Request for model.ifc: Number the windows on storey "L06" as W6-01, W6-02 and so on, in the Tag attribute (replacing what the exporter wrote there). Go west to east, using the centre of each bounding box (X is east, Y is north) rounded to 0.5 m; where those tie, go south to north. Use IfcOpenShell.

First a look at what the model holds.

```python
import ifcopenshell
import ifcopenshell.util.element
import ifcopenshell.util.placement

model = ifcopenshell.open("model.ifc")
print(model.schema)
storey = next(s for s in model.by_type("IfcBuildingStorey") if s.Name == "L06")
windows = [e for e in ifcopenshell.util.element.get_decomposition(storey) if e.is_a("IfcWindow")]
for e in sorted(windows, key=lambda e: e.id()):
    origin = ifcopenshell.util.placement.get_local_placement(e.ObjectPlacement)[:3, 3]
    print(e.id(), e.Tag, e.Name, origin.round(2) + 0.0, sep=" | ")
```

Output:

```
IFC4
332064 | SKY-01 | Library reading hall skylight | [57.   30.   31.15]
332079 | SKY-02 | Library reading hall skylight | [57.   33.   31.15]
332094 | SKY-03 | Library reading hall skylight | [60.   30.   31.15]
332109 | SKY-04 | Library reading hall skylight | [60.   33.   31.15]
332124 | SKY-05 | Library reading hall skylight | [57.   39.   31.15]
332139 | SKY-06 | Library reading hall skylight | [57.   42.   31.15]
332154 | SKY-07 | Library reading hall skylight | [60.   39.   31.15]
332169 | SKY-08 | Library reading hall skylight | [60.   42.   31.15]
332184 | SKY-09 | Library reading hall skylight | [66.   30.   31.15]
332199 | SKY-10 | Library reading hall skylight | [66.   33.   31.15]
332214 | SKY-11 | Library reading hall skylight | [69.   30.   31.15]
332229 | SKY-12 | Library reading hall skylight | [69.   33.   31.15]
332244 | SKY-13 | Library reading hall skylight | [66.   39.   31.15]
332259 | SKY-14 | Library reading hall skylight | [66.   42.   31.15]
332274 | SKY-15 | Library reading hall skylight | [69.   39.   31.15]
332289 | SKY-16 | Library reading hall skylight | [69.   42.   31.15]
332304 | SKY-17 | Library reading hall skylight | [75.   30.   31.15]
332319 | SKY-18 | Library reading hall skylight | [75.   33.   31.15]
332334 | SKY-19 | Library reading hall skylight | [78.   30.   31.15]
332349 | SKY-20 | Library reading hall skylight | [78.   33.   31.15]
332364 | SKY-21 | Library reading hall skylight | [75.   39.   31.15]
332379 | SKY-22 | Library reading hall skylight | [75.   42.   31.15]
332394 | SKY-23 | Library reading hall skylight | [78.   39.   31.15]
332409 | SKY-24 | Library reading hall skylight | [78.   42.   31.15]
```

```python
import ifcopenshell
import ifcopenshell.geom
import ifcopenshell.util.element
import ifcopenshell.util.shape

model = ifcopenshell.open("model.ifc")
settings = ifcopenshell.geom.settings()
settings.set("use-world-coords", True)


def centre(element):
    shape = ifcopenshell.geom.create_shape(settings, element)
    return ifcopenshell.util.shape.get_bbox_centroid(shape.geometry)


storey = next(s for s in model.by_type("IfcBuildingStorey") if s.Name == "L06")
windows = [e for e in ifcopenshell.util.element.get_decomposition(storey) if e.is_a("IfcWindow")]

# Insertion points can sit at a corner or the storey origin, so sort by the geometry (in metres).
centres = {e: centre(e) for e in windows}
windows.sort(key=lambda e: (round(centres[e][0] / 0.5), centres[e][1]))

for i, e in enumerate(windows, start=1):
    number = f"W6-{i:02d}"
    e.Tag = number
    print(e.id(), number)

model.write("model_rev.ifc")
```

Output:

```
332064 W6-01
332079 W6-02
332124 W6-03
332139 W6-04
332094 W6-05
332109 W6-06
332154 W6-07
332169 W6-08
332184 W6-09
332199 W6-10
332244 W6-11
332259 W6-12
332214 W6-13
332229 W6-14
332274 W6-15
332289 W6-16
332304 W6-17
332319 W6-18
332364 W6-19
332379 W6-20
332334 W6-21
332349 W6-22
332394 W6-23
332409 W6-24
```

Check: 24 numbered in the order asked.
